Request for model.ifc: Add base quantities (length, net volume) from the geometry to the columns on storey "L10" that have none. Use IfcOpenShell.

First a look at what the model holds.

```python
import ifcopenshell
import ifcopenshell.util.element
import ifcopenshell.util.unit

model = ifcopenshell.open("model.ifc")
print(model.schema)
for unit_type in ("LENGTHUNIT", "AREAUNIT", "VOLUMEUNIT"):
    print(unit_type, ifcopenshell.util.unit.calculate_unit_scale(model, unit_type))
storey = next(s for s in model.by_type("IfcBuildingStorey") if s.Name == "L10")
columns = [e for e in ifcopenshell.util.element.get_decomposition(storey) if e.is_a("IfcColumn")]
for e in sorted(columns, key=lambda e: e.id()):
    print(e.id(), e.is_a(), e.Name, list(ifcopenshell.util.element.get_psets(e, qtos_only=True)), sep=" | ")
```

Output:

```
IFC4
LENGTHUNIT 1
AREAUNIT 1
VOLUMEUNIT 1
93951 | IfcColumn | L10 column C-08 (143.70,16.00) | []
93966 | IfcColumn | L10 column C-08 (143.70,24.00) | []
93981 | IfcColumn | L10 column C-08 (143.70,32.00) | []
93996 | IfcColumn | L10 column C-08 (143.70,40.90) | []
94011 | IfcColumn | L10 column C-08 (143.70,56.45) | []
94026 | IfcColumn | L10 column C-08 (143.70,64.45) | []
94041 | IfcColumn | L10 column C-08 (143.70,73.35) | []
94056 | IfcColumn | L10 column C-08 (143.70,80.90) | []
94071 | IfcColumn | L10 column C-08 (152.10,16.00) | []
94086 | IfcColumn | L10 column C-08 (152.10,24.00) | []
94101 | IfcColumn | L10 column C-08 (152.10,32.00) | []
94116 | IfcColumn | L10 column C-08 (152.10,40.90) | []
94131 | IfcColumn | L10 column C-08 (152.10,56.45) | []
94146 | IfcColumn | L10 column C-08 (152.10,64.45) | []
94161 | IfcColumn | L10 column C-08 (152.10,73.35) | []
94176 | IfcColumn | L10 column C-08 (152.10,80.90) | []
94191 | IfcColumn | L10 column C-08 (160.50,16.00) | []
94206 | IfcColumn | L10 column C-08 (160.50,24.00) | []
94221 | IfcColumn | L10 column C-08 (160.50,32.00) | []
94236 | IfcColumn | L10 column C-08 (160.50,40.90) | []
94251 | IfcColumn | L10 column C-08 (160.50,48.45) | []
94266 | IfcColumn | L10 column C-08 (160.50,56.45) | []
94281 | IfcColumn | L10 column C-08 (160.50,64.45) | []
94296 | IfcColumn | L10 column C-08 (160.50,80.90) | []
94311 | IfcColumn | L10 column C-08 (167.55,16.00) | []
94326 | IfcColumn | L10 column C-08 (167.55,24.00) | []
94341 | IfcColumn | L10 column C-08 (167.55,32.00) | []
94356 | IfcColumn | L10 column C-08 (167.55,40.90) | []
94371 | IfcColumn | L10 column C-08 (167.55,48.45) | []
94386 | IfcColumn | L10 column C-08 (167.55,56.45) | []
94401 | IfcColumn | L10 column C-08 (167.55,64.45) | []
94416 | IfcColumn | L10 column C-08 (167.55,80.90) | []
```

```python
import ifcopenshell
import ifcopenshell.api.pset
import ifcopenshell.geom
import ifcopenshell.util.element
import ifcopenshell.util.shape
import ifcopenshell.util.unit

model = ifcopenshell.open("model.ifc")
unit_scale = ifcopenshell.util.unit.calculate_unit_scale(model)
volume_scale = ifcopenshell.util.unit.calculate_unit_scale(model, "VOLUMEUNIT")
settings = ifcopenshell.geom.settings()

storey = next(s for s in model.by_type("IfcBuildingStorey") if s.Name == "L10")
columns = [e for e in ifcopenshell.util.element.get_decomposition(storey) if e.is_a("IfcColumn")]

for e in sorted(columns, key=lambda e: e.id()):
    if ifcopenshell.util.element.get_psets(e, qtos_only=True, should_inherit=False):
        continue
    # Geometry comes back in metres, in the element's own axes.
    shape = ifcopenshell.geom.create_shape(settings, e)
    values = {
        "Length": ifcopenshell.util.shape.get_z(shape.geometry) / unit_scale,
        "NetVolume": ifcopenshell.util.shape.get_volume(shape.geometry) / volume_scale,
    }
    qto = ifcopenshell.api.pset.add_qto(model, product=e, name="Qto_ColumnBaseQuantities")
    ifcopenshell.api.pset.edit_qto(model, qto=qto, properties=values)
    print(e.id(), {k: round(v, 3) for k, v in values.items()})

model.write("model_edited.ifc")
```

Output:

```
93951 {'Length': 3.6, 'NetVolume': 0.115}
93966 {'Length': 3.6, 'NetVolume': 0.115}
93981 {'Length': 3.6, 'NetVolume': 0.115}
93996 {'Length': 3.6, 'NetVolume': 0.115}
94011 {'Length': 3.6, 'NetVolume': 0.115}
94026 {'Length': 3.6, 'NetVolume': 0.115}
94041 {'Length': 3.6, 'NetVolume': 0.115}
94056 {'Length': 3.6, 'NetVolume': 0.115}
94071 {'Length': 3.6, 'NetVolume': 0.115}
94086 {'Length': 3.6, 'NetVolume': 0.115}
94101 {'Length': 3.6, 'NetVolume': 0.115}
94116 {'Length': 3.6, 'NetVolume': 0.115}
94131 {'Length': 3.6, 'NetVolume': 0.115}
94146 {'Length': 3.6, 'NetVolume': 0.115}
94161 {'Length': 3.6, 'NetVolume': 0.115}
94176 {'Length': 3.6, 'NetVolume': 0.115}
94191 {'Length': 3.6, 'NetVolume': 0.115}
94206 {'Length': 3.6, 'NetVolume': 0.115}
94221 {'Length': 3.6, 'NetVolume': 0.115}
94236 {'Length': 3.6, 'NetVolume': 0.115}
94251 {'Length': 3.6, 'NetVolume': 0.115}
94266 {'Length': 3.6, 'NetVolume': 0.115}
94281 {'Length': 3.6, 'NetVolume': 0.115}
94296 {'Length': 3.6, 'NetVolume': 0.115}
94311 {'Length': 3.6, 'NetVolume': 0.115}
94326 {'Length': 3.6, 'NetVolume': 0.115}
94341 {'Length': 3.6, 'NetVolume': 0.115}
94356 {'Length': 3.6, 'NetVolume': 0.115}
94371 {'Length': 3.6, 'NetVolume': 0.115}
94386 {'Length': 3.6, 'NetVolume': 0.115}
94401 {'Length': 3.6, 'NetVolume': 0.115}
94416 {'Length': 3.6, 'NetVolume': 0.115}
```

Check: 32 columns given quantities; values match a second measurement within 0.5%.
